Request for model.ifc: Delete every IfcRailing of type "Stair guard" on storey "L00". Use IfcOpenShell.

First a look at what the model holds.

```python
import ifcopenshell
import ifcopenshell.util.element

model = ifcopenshell.open("model.ifc")
print(model.schema)
storey = next(s for s in model.by_type("IfcBuildingStorey") if s.Name == "L00")
railings = [e for e in ifcopenshell.util.element.get_decomposition(storey) if e.is_a("IfcRailing")]
seen = {}
for e in railings:
    element_type = ifcopenshell.util.element.get_type(e)
    name = element_type.Name if element_type not in (None, e) else None
    seen[name] = seen.get(name, 0) + 1
for name, count in sorted(seen.items(), key=str):
    print(count, "x", name)
```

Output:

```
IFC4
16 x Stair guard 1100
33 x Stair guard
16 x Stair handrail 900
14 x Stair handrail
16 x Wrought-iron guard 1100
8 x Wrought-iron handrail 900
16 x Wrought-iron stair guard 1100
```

```python
import ifcopenshell
import ifcopenshell.api.root
import ifcopenshell.util.element

model = ifcopenshell.open("model.ifc")

storey = next(s for s in model.by_type("IfcBuildingStorey") if s.Name == "L00")
railings = [e for e in ifcopenshell.util.element.get_decomposition(storey) if e.is_a("IfcRailing")]
targets = [e for e in railings if (t := ifcopenshell.util.element.get_type(e)) not in (None, e) and t.Name == "Stair guard"]

for e in targets:
    ifcopenshell.api.root.remove_product(model, product=e)
print(len(targets), "removed")

model.write("model_v2.ifc")
```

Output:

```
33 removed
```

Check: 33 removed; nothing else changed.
